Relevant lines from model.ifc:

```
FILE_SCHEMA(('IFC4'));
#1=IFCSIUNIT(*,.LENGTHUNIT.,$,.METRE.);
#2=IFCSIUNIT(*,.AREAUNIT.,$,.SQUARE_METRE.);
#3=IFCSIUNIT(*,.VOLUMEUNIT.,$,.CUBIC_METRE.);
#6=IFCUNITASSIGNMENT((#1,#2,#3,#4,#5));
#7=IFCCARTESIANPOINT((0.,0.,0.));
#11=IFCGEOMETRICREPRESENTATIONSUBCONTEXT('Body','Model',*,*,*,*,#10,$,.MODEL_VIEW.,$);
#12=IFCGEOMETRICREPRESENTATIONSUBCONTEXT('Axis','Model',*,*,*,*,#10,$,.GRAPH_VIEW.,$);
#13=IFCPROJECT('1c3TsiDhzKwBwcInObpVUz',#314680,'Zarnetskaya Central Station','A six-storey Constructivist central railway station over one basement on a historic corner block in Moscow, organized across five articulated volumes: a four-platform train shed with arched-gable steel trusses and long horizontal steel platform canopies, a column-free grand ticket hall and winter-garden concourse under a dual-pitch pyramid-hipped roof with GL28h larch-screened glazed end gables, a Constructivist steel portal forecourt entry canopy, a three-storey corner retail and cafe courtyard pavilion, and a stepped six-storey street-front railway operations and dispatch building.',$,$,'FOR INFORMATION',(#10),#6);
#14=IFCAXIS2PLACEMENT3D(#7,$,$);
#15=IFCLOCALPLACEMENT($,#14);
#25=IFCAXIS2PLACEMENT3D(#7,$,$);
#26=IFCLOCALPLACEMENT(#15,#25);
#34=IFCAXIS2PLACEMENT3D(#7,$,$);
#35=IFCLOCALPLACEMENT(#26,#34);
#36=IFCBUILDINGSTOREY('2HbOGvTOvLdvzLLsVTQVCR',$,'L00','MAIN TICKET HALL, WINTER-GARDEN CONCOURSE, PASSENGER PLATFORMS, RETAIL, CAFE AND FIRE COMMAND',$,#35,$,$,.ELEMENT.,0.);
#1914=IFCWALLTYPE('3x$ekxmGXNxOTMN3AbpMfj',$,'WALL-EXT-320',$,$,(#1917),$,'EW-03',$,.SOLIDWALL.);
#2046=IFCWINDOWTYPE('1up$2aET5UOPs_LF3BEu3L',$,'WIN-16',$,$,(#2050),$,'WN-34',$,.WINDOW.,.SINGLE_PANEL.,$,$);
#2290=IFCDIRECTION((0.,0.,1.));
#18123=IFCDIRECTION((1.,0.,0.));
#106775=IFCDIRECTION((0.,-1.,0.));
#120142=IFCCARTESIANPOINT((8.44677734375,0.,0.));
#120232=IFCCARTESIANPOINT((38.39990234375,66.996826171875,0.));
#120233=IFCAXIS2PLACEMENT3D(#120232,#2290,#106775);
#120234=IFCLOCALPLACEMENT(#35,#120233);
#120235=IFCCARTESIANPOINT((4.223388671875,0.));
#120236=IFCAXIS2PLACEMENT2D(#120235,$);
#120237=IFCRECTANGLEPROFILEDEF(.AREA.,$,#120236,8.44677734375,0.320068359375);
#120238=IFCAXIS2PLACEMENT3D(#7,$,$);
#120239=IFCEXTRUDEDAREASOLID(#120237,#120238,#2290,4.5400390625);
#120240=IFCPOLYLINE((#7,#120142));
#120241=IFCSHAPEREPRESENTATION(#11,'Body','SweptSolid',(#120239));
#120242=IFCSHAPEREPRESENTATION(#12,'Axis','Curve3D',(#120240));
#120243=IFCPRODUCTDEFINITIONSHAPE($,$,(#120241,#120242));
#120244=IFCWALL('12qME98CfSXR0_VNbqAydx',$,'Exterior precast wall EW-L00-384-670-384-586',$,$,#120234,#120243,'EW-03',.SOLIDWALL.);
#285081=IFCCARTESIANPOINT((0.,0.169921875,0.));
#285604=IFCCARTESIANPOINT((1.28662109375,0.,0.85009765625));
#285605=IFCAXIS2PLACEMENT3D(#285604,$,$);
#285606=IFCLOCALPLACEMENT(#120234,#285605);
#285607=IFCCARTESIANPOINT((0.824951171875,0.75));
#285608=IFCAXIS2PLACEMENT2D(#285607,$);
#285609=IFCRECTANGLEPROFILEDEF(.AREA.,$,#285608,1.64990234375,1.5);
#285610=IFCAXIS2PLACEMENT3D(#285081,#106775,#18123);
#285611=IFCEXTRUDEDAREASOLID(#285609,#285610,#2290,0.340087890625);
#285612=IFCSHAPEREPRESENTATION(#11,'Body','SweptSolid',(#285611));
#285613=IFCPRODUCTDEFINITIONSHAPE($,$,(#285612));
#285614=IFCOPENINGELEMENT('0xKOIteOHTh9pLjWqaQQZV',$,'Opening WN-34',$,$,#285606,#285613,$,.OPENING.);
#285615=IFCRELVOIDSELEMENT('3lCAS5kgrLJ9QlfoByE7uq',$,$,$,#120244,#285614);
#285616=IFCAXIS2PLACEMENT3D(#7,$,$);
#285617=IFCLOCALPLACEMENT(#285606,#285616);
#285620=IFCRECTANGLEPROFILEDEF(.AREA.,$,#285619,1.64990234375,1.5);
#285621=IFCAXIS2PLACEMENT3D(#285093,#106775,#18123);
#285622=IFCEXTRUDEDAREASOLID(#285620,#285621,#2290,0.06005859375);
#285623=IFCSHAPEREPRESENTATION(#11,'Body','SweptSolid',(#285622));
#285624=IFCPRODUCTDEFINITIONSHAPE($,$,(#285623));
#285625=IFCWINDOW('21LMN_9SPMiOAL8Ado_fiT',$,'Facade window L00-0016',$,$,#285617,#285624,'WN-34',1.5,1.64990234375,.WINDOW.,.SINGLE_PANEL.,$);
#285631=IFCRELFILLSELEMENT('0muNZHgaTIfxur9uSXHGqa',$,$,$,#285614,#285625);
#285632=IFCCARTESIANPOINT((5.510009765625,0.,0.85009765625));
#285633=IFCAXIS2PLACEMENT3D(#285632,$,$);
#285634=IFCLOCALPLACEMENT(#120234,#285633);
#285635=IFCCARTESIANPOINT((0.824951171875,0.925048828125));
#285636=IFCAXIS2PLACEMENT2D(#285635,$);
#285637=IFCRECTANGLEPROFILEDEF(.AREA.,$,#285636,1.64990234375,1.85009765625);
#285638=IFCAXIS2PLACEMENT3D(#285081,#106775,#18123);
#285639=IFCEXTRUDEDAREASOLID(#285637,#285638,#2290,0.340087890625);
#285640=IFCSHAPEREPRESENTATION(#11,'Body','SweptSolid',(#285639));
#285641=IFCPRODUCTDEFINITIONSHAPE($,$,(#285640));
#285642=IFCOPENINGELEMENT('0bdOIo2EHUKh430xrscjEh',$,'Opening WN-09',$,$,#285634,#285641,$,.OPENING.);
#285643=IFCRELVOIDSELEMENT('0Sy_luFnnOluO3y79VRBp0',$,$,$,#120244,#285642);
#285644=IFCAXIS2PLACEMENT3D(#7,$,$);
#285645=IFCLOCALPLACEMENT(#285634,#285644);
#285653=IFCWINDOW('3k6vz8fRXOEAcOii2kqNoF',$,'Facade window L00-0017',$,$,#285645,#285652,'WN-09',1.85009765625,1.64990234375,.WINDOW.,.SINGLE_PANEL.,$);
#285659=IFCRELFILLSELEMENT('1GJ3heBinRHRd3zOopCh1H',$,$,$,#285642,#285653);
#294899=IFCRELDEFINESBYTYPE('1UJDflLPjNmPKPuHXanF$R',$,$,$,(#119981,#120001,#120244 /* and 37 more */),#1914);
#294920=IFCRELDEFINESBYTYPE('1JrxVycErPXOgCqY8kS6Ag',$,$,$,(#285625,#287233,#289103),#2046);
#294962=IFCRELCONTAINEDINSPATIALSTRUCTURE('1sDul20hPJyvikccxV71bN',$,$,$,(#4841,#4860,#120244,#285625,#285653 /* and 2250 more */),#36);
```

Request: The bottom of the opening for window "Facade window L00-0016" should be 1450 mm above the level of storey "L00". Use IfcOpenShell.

```python
import numpy as np
import ifcopenshell
import ifcopenshell.api.geometry
import ifcopenshell.geom
import ifcopenshell.util.element
import ifcopenshell.util.placement
import ifcopenshell.util.shape
import ifcopenshell.util.unit

model = ifcopenshell.open("model.ifc")
unit_scale = ifcopenshell.util.unit.calculate_unit_scale(model)

window = model.by_guid("21LMN_9SPMiOAL8Ado_fiT")
opening = window.FillsVoids[0].RelatingOpeningElement
storey = ifcopenshell.util.element.get_container(window, ifc_class="IfcBuildingStorey")
level = ifcopenshell.util.placement.get_local_placement(storey.ObjectPlacement)[2, 3]

# The opening's origin need not be at the sill, so measure its lowest point.
shape = ifcopenshell.geom.create_shape(ifcopenshell.geom.settings(), opening)
bottom = ifcopenshell.util.shape.get_shape_bottom_elevation(shape, shape.geometry) / unit_scale
dz = level + 1.45 / unit_scale - bottom

shift = np.array([0.0, 0.0, dz])
# The window is placed relative to its opening, so it follows when the opening moves.
matrix = ifcopenshell.util.placement.get_local_placement(opening.ObjectPlacement)
matrix[:3, 3] += shift
ifcopenshell.api.geometry.edit_object_placement(
    model, product=opening, matrix=matrix, is_si=False, should_transform_children=True
)

print(f"moved by {dz * unit_scale:+.3f} m")

model.write("model_v2.ifc")
```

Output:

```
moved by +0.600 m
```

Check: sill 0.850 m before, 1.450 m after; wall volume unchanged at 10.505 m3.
